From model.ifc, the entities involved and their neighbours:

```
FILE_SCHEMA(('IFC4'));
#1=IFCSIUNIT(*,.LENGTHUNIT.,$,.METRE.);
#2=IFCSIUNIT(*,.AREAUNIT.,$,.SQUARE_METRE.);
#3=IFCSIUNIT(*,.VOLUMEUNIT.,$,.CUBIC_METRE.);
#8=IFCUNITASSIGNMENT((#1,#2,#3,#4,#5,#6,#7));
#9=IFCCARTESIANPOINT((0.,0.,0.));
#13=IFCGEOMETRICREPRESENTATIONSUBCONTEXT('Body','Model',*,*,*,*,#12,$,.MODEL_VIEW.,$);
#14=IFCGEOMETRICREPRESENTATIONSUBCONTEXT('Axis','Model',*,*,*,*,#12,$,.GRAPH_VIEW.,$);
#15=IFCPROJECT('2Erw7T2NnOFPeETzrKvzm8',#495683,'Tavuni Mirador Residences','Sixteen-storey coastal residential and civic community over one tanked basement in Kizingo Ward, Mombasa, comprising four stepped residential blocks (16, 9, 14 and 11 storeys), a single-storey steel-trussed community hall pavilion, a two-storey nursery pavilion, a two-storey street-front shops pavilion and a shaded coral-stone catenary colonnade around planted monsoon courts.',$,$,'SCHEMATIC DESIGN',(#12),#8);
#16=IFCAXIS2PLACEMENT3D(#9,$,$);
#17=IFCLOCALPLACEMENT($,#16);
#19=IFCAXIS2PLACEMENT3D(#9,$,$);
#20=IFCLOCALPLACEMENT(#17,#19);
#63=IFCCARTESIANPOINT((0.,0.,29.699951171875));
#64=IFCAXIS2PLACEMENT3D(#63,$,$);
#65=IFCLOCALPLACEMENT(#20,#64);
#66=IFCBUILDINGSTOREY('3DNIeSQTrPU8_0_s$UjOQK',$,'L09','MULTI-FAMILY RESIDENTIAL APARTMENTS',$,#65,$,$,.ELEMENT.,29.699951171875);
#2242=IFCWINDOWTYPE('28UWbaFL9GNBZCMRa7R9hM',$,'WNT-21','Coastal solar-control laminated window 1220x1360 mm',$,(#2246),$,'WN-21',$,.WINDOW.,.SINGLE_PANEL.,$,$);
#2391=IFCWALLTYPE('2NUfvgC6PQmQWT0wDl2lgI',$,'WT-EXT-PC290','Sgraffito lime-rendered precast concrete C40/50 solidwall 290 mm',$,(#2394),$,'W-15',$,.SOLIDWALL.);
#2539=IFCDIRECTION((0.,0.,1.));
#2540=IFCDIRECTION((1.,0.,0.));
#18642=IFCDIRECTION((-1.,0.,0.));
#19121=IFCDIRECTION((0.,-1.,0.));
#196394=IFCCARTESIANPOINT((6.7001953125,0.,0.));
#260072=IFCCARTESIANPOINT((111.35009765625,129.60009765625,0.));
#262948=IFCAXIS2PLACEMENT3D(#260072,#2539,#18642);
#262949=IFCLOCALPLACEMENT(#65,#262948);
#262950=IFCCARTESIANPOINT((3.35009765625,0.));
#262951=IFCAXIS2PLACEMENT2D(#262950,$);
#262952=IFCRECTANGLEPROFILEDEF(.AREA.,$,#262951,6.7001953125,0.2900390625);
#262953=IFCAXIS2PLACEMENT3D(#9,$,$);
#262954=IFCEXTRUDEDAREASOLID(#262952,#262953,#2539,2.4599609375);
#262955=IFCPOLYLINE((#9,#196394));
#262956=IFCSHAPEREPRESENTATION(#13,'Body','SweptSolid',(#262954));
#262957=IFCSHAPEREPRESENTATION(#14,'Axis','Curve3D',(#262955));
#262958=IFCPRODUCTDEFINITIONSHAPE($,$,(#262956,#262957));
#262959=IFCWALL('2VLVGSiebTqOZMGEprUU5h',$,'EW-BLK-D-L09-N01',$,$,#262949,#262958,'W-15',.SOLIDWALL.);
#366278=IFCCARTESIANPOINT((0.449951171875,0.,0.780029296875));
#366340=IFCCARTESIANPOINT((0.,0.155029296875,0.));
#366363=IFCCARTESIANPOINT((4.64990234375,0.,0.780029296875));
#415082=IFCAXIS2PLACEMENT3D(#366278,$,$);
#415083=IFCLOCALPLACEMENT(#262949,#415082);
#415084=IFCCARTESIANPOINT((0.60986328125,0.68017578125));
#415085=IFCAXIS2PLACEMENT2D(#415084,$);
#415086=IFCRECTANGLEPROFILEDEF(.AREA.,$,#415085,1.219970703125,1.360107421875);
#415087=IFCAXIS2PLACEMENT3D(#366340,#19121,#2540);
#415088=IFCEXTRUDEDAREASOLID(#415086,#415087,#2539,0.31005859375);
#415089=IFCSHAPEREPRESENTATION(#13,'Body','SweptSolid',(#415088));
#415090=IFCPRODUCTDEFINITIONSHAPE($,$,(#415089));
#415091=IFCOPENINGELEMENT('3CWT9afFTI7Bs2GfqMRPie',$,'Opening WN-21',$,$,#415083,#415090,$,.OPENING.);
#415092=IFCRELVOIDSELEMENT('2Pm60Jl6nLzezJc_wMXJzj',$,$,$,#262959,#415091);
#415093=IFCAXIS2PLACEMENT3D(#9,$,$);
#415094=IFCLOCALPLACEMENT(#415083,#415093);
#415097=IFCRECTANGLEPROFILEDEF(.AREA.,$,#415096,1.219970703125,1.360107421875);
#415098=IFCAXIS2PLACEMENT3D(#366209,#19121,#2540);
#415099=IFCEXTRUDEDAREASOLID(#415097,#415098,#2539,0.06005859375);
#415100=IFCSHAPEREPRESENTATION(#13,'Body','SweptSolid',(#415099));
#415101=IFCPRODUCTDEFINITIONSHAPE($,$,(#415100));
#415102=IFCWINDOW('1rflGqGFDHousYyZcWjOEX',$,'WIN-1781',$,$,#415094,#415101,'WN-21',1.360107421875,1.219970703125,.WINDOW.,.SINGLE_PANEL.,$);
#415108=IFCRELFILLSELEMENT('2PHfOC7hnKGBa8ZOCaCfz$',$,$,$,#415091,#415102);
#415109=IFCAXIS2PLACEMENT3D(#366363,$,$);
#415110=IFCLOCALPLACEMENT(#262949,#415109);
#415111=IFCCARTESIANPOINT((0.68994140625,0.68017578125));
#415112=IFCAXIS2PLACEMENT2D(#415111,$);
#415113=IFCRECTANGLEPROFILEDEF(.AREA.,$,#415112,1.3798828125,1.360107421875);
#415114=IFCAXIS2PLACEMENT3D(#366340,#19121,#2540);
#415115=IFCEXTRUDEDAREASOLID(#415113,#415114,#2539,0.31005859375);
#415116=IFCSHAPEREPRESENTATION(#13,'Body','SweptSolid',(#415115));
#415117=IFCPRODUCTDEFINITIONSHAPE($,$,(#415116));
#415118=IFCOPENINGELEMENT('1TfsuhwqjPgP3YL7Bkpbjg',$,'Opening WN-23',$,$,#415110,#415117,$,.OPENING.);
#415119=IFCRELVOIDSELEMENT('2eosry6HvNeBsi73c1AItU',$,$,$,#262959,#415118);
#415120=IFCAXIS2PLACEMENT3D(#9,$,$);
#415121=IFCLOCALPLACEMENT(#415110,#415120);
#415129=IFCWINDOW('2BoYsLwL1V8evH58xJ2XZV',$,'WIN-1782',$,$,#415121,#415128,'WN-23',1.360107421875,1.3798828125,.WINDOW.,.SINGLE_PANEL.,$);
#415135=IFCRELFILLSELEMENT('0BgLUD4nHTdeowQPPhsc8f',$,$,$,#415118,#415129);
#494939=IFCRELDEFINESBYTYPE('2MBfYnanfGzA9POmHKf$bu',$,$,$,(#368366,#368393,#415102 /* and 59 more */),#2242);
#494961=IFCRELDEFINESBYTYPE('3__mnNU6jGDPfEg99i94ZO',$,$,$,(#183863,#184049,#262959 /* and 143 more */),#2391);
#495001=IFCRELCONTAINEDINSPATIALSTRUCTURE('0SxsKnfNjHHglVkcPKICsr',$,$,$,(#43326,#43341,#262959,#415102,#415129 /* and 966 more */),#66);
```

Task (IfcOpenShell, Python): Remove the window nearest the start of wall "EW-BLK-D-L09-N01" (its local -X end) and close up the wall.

```python
import ifcopenshell
import ifcopenshell.api.feature
import ifcopenshell.api.root
import ifcopenshell.geom
import ifcopenshell.util.shape

model = ifcopenshell.open("model.ifc")
settings = ifcopenshell.geom.settings()


def volume(element):
    """Net volume in cubic metres, openings subtracted."""
    shape = ifcopenshell.geom.create_shape(settings, element)
    return ifcopenshell.util.shape.get_volume(shape.geometry)


window = model.by_guid("1rflGqGFDHousYyZcWjOEX")
opening = window.FillsVoids[0].RelatingOpeningElement
wall = opening.VoidsElements[0].RelatingBuildingElement
before = volume(wall)

ifcopenshell.api.root.remove_product(model, product=window)
ifcopenshell.api.feature.remove_feature(model, feature=opening)

after = volume(wall)

print(f"wall volume {before:.3f} -> {after:.3f} m3")

model.write("model_rev.ifc")
```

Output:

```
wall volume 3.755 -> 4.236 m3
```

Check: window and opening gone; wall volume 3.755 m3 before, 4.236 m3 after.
